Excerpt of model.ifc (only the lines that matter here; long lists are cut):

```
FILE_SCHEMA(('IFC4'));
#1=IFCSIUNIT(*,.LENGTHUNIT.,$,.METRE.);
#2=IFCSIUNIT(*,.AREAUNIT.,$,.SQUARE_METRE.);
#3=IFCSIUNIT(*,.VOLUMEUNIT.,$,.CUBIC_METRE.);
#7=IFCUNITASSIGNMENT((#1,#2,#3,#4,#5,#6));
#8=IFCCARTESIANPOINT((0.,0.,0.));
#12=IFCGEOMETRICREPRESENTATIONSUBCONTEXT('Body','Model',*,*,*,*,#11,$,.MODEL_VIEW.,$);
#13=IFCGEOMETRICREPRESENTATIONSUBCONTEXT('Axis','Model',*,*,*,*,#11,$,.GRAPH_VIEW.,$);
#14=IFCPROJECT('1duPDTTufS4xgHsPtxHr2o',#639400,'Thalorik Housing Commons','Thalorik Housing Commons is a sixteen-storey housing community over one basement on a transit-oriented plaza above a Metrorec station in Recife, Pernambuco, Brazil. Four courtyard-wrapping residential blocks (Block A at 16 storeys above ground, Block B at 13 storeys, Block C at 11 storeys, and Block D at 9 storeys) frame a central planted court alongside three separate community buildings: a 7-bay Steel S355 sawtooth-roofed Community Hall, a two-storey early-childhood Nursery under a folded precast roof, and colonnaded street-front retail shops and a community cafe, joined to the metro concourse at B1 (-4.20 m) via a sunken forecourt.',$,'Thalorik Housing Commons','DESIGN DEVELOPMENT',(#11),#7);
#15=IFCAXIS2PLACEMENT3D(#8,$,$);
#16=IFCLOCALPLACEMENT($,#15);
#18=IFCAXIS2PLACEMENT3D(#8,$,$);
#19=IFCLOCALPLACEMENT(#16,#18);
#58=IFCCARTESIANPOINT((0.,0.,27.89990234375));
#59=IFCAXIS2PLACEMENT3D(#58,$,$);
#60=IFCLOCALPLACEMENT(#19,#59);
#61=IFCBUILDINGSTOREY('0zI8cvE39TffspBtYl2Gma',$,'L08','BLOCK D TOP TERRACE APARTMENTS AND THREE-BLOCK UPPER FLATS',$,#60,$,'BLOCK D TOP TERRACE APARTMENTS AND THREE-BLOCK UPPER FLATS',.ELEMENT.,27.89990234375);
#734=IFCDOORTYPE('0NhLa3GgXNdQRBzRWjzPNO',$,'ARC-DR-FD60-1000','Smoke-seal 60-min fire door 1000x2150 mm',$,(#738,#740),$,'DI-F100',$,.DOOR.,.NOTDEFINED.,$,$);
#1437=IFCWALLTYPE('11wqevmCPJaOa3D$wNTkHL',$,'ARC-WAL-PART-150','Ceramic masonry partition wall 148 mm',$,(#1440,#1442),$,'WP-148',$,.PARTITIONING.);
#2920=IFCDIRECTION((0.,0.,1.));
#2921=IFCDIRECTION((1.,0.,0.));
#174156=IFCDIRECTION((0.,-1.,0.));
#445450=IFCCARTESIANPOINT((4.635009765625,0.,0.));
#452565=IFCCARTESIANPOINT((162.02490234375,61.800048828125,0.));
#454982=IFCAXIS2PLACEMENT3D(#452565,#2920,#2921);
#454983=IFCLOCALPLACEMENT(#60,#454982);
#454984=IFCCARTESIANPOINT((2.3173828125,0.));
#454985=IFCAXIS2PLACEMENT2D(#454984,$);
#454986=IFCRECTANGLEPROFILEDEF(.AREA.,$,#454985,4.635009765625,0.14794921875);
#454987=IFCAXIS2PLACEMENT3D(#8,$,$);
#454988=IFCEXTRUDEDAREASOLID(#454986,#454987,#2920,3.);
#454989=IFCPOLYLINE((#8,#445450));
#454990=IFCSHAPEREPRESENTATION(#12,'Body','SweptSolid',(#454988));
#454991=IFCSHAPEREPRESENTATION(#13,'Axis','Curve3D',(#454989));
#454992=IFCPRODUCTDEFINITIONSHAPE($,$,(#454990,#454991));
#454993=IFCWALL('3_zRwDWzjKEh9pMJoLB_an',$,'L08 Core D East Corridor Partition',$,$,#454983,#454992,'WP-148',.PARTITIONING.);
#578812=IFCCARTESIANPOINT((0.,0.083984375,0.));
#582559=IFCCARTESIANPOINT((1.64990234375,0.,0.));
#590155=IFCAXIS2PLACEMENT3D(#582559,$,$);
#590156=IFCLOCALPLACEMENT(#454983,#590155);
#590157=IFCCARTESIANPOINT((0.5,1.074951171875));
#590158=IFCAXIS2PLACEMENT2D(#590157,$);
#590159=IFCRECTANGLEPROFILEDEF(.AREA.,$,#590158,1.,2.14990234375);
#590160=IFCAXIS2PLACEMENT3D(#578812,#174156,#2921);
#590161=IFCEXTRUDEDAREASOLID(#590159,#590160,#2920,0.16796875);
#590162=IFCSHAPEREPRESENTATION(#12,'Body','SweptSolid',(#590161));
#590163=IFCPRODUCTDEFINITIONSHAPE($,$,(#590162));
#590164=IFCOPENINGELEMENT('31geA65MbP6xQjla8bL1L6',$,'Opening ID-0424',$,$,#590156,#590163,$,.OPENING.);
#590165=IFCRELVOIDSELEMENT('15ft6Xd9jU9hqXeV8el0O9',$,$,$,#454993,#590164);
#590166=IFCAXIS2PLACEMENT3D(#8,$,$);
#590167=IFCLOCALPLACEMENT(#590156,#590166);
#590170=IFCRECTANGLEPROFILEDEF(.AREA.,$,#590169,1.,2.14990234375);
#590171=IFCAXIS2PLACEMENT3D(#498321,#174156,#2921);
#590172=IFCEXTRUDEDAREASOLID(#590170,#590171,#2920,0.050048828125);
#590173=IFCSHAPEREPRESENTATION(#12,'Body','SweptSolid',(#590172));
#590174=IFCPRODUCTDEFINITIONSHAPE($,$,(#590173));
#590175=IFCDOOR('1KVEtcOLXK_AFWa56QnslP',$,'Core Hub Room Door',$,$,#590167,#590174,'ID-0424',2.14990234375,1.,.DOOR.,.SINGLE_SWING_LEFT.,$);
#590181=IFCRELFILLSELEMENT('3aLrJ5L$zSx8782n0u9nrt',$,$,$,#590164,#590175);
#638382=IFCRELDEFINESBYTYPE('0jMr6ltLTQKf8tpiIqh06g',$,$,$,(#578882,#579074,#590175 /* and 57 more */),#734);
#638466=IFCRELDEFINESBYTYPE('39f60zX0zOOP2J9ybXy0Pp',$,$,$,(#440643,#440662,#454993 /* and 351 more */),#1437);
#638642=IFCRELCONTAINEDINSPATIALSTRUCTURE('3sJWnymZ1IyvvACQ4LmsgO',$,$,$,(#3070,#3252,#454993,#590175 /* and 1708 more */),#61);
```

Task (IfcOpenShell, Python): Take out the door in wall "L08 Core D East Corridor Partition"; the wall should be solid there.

```python
import ifcopenshell
import ifcopenshell.api.feature
import ifcopenshell.api.root
import ifcopenshell.geom
import ifcopenshell.util.shape

model = ifcopenshell.open("model.ifc")
settings = ifcopenshell.geom.settings()


def volume(element):
    """Net volume in cubic metres, openings subtracted."""
    shape = ifcopenshell.geom.create_shape(settings, element)
    return ifcopenshell.util.shape.get_volume(shape.geometry)


door = model.by_id(590175)
opening = door.FillsVoids[0].RelatingOpeningElement
wall = opening.VoidsElements[0].RelatingBuildingElement
before = volume(wall)

ifcopenshell.api.root.remove_product(model, product=door)
ifcopenshell.api.feature.remove_feature(model, feature=opening)

after = volume(wall)

print(f"wall volume {before:.3f} -> {after:.3f} m3")

model.write("model_edited.ifc")
```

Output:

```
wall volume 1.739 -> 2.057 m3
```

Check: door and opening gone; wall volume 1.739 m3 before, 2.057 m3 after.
